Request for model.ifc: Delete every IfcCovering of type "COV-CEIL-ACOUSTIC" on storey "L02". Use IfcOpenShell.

First a look at what the model holds.

```python
import ifcopenshell
import ifcopenshell.util.element

model = ifcopenshell.open("model.ifc")
print(model.schema)
storey = next(s for s in model.by_type("IfcBuildingStorey") if s.Name == "L02")
coverings = [e for e in ifcopenshell.util.element.get_decomposition(storey) if e.is_a("IfcCovering")]
seen = {}
for e in coverings:
    element_type = ifcopenshell.util.element.get_type(e)
    name = element_type.Name if element_type not in (None, e) else None
    seen[name] = seen.get(name, 0) + 1
for name, count in sorted(seen.items(), key=str):
    print(count, "x", name)
```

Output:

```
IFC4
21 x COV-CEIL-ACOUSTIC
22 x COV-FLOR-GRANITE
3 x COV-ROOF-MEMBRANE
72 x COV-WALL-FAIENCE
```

```python
import ifcopenshell
import ifcopenshell.api.root
import ifcopenshell.util.element

model = ifcopenshell.open("model.ifc")

storey = next(s for s in model.by_type("IfcBuildingStorey") if s.Name == "L02")
coverings = [e for e in ifcopenshell.util.element.get_decomposition(storey) if e.is_a("IfcCovering")]
targets = [e for e in coverings if (t := ifcopenshell.util.element.get_type(e)) not in (None, e) and t.Name == "COV-CEIL-ACOUSTIC"]

for e in targets:
    ifcopenshell.api.root.remove_product(model, product=e)
print(len(targets), "removed")

model.write("model-out.ifc")
```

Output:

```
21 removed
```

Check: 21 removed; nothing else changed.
